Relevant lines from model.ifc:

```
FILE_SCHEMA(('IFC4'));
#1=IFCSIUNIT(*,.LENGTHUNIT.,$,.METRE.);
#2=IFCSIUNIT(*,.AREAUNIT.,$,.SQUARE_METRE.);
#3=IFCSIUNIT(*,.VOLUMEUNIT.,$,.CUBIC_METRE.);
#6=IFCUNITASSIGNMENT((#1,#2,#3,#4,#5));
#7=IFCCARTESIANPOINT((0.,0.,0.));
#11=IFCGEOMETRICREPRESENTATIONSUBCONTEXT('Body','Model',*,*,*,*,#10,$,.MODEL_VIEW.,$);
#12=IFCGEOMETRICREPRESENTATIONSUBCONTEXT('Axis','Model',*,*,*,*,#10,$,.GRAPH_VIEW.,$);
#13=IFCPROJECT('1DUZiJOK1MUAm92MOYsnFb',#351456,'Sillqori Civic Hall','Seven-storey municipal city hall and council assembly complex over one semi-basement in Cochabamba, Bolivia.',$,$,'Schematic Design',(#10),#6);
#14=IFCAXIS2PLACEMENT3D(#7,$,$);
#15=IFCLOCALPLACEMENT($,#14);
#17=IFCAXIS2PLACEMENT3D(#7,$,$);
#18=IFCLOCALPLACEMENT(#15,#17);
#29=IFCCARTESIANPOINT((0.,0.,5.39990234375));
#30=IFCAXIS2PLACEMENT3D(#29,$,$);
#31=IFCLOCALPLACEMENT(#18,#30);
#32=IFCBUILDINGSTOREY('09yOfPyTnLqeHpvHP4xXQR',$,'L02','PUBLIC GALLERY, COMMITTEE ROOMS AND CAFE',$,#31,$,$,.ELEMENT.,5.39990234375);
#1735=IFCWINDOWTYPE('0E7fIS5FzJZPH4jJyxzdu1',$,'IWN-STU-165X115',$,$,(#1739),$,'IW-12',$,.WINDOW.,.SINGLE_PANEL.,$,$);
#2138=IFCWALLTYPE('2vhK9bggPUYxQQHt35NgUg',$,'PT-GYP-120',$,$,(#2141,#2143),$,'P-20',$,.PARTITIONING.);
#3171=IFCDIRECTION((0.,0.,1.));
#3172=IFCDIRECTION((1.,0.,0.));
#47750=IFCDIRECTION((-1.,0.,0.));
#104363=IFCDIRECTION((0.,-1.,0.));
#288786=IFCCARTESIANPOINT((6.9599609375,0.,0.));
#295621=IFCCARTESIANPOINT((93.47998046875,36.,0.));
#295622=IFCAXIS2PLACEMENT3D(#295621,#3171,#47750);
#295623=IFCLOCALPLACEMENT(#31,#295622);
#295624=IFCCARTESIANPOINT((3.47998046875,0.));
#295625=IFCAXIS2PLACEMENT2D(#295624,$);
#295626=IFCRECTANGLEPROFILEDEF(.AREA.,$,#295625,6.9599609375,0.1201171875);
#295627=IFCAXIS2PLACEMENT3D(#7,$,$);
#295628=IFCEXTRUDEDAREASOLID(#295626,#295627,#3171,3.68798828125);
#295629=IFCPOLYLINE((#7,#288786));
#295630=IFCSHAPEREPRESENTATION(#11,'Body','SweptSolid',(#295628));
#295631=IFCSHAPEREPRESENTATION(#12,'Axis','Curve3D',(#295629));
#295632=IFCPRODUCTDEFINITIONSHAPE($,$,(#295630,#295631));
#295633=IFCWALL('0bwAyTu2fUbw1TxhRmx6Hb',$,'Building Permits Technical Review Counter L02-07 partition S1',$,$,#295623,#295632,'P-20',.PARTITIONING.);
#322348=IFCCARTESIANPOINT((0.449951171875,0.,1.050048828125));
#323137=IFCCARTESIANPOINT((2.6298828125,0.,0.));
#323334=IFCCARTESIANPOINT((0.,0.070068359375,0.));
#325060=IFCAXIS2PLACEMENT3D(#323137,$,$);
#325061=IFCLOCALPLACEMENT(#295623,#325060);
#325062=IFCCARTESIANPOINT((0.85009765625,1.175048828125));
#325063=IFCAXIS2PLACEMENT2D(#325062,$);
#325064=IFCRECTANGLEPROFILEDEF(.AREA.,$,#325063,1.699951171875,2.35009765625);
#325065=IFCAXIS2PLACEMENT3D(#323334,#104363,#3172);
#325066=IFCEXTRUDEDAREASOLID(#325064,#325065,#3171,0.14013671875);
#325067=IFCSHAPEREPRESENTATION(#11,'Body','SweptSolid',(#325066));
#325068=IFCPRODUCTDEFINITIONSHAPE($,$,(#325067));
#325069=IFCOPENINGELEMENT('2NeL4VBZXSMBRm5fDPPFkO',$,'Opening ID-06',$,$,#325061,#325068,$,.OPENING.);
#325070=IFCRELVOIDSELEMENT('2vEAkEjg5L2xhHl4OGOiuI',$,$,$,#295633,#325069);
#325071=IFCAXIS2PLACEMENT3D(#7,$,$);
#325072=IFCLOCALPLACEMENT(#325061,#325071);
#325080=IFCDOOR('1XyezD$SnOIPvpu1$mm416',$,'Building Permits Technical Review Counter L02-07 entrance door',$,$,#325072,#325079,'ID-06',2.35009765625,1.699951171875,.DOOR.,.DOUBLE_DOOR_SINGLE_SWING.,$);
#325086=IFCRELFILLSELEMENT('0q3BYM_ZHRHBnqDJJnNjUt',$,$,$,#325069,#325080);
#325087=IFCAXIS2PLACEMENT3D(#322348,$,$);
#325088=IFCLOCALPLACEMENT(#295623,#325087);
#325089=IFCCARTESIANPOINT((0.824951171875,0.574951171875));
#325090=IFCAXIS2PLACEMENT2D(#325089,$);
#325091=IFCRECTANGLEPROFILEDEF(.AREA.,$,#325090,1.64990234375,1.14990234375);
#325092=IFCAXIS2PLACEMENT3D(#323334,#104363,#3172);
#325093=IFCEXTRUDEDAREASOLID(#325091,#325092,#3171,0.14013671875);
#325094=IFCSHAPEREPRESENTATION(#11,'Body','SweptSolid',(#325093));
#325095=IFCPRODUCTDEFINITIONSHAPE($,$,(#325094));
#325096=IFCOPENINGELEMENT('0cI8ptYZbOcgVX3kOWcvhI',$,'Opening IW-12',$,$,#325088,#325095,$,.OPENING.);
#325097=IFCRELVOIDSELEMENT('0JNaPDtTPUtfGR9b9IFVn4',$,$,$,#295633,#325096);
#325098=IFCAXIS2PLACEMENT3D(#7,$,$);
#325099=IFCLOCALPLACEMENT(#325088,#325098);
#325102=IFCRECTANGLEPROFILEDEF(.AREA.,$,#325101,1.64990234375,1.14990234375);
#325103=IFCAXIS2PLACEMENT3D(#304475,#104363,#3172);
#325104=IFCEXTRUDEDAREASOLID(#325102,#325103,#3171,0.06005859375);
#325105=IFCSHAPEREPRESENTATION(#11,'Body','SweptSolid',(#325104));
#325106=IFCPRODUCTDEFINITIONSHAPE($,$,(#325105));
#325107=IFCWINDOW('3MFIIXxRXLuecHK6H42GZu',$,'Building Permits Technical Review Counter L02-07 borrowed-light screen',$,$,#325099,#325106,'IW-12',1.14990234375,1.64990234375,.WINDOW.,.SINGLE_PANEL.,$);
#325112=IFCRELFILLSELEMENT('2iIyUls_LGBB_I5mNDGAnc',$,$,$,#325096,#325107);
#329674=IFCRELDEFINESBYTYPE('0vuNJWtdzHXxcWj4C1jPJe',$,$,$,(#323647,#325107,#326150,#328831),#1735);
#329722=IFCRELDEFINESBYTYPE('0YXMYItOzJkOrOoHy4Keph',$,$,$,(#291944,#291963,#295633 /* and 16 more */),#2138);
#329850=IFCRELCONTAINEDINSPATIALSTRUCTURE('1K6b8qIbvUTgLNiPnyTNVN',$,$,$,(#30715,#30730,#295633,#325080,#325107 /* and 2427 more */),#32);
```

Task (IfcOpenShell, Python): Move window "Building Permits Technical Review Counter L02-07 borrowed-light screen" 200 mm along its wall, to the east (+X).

```python
import ifcopenshell
import ifcopenshell.api.geometry
import ifcopenshell.util.placement

model = ifcopenshell.open("model.ifc")

window = model.by_guid("3MFIIXxRXLuecHK6H42GZu")
opening = window.FillsVoids[0].RelatingOpeningElement
wall = opening.VoidsElements[0].RelatingBuildingElement

wall_matrix = ifcopenshell.util.placement.get_local_placement(wall.ObjectPlacement)
shift = wall_matrix[:3, 0] * -0.2
before = ifcopenshell.util.placement.get_local_placement(window.ObjectPlacement)[:3, 3].copy()

# The window is placed relative to its opening, so it follows when the opening moves.
matrix = ifcopenshell.util.placement.get_local_placement(opening.ObjectPlacement)
matrix[:3, 3] += shift
ifcopenshell.api.geometry.edit_object_placement(
    model, product=opening, matrix=matrix, is_si=False, should_transform_children=True
)

after = ifcopenshell.util.placement.get_local_placement(window.ObjectPlacement)[:3, 3]
print("window moved by", (after - before).round(3) + 0.0)

model.write("model_v2.ifc")
```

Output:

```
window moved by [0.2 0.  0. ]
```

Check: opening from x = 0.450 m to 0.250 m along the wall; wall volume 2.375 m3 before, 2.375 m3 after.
